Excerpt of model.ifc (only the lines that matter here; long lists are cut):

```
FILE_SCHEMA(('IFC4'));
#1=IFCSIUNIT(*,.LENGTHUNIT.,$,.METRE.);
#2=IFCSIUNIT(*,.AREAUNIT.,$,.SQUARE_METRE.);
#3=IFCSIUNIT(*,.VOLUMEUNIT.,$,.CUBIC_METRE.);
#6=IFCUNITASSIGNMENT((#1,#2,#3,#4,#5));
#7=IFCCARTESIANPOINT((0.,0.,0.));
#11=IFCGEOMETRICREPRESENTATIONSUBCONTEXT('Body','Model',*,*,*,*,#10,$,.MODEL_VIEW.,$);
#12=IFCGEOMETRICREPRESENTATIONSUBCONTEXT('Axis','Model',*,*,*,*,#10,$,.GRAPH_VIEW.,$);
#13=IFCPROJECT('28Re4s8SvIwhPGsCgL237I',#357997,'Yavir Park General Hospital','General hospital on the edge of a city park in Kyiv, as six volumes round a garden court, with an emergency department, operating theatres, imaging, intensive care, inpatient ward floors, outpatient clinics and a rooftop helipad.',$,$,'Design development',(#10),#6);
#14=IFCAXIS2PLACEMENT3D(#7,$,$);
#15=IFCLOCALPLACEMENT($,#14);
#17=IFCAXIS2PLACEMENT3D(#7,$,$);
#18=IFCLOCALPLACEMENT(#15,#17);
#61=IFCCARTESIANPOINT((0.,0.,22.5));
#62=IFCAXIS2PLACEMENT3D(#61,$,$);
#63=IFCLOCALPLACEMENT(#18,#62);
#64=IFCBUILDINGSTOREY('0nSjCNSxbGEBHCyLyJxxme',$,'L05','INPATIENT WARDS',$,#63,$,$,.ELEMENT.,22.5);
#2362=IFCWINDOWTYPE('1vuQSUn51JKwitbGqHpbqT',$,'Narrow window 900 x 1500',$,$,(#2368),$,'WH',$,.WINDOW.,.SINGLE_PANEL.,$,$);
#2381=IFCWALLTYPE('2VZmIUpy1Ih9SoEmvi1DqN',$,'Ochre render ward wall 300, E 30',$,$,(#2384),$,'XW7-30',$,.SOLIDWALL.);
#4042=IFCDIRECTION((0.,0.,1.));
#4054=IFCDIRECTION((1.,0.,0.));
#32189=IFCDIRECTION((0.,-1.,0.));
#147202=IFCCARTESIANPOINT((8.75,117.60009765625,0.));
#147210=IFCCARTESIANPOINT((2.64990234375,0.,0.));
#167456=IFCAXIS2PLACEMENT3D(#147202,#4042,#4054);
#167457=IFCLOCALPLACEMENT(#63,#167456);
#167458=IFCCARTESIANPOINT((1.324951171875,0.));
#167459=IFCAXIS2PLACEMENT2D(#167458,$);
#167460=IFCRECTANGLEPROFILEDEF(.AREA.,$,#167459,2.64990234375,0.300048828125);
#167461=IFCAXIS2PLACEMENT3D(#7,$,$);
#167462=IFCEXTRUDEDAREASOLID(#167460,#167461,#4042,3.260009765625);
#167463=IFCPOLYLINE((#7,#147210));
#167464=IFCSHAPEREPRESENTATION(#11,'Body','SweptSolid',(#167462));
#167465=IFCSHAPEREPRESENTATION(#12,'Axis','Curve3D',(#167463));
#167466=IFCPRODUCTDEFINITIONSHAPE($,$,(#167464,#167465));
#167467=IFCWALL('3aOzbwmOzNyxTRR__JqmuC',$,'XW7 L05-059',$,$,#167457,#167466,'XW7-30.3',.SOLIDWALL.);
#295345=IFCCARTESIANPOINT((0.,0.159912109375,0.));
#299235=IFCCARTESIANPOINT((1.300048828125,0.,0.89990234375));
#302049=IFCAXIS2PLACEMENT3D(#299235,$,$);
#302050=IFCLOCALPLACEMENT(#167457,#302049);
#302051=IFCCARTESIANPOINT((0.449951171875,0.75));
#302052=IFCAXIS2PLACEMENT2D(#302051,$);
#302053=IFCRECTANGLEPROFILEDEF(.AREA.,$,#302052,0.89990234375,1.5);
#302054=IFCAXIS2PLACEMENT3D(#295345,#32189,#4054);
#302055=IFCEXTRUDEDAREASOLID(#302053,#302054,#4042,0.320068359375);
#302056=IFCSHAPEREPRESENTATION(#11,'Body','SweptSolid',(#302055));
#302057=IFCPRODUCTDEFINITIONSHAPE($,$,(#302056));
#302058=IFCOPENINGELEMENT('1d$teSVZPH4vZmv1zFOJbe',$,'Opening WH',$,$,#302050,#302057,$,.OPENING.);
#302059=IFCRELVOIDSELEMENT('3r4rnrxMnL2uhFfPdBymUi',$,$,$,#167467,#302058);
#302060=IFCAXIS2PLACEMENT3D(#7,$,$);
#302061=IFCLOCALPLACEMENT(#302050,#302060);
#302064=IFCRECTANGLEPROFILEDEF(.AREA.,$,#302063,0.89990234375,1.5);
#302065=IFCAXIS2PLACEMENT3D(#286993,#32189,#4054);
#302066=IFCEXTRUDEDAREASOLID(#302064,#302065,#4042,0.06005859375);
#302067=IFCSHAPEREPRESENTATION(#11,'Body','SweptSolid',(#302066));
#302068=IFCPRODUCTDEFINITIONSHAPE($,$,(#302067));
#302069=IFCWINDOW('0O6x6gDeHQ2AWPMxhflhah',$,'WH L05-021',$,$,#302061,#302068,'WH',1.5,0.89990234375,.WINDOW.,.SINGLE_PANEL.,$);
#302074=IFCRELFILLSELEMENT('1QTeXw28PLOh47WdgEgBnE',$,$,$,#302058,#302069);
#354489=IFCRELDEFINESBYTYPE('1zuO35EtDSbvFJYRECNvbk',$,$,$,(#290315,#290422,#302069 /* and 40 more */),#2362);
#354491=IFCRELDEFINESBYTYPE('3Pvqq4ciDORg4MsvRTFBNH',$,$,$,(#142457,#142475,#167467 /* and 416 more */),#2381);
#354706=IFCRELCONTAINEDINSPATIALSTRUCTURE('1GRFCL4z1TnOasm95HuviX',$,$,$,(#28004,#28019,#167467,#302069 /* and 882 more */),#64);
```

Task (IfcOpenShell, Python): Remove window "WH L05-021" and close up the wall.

```python
import ifcopenshell
import ifcopenshell.api.feature
import ifcopenshell.api.root
import ifcopenshell.geom
import ifcopenshell.util.shape

model = ifcopenshell.open("model.ifc")
settings = ifcopenshell.geom.settings()


def volume(element):
    """Net volume in cubic metres, openings subtracted."""
    shape = ifcopenshell.geom.create_shape(settings, element)
    return ifcopenshell.util.shape.get_volume(shape.geometry)


window = model.by_guid("0O6x6gDeHQ2AWPMxhflhah")
opening = window.FillsVoids[0].RelatingOpeningElement
wall = opening.VoidsElements[0].RelatingBuildingElement
before = volume(wall)

ifcopenshell.api.root.remove_product(model, product=window)
ifcopenshell.api.feature.remove_feature(model, feature=opening)

after = volume(wall)

print(f"wall volume {before:.3f} -> {after:.3f} m3")

model.write("model_edited.ifc")
```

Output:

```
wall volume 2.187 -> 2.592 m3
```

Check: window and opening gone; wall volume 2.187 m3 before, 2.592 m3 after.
